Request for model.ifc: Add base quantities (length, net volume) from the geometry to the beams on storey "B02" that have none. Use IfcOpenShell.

First a look at what the model holds.

```python
import ifcopenshell
import ifcopenshell.util.element
import ifcopenshell.util.unit

model = ifcopenshell.open("model.ifc")
print(model.schema)
for unit_type in ("LENGTHUNIT", "AREAUNIT", "VOLUMEUNIT"):
    print(unit_type, ifcopenshell.util.unit.calculate_unit_scale(model, unit_type))
storey = next(s for s in model.by_type("IfcBuildingStorey") if s.Name == "B02")
beams = [e for e in ifcopenshell.util.element.get_decomposition(storey) if e.is_a("IfcBeam")]
for e in sorted(beams, key=lambda e: e.id()):
    print(e.id(), e.is_a(), e.Name, list(ifcopenshell.util.element.get_psets(e, qtos_only=True)), sep=" | ")
```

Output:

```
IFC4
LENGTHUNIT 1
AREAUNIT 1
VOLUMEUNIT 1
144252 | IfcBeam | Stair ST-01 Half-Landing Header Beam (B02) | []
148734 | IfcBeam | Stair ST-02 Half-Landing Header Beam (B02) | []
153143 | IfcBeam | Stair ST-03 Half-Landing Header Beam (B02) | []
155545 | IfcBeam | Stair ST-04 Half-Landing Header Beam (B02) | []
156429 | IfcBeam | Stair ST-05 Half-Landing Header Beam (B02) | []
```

```python
import ifcopenshell
import ifcopenshell.api.pset
import ifcopenshell.geom
import ifcopenshell.util.element
import ifcopenshell.util.shape
import ifcopenshell.util.unit

model = ifcopenshell.open("model.ifc")
unit_scale = ifcopenshell.util.unit.calculate_unit_scale(model)
volume_scale = ifcopenshell.util.unit.calculate_unit_scale(model, "VOLUMEUNIT")
settings = ifcopenshell.geom.settings()

storey = next(s for s in model.by_type("IfcBuildingStorey") if s.Name == "B02")
beams = [e for e in ifcopenshell.util.element.get_decomposition(storey) if e.is_a("IfcBeam")]

for e in sorted(beams, key=lambda e: e.id()):
    if ifcopenshell.util.element.get_psets(e, qtos_only=True, should_inherit=False):
        continue
    # Geometry comes back in metres, in the element's own axes.
    shape = ifcopenshell.geom.create_shape(settings, e)
    values = {
        "Length": ifcopenshell.util.shape.get_max_xyz(shape.geometry) / unit_scale,
        "NetVolume": ifcopenshell.util.shape.get_volume(shape.geometry) / volume_scale,
    }
    qto = ifcopenshell.api.pset.add_qto(model, product=e, name="Qto_BeamBaseQuantities")
    ifcopenshell.api.pset.edit_qto(model, qto=qto, properties=values)
    print(e.id(), {k: round(v, 3) for k, v in values.items()})

model.write("model_updated.ifc")
```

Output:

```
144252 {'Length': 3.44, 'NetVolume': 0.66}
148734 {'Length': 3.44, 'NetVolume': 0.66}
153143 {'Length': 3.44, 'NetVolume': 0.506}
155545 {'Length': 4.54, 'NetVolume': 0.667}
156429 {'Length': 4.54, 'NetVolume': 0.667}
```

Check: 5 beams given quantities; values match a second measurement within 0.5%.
